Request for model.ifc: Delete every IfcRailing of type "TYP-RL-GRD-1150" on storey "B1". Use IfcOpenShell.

First a look at what the model holds.

```python
import ifcopenshell
import ifcopenshell.util.element

model = ifcopenshell.open("model.ifc")
print(model.schema)
storey = next(s for s in model.by_type("IfcBuildingStorey") if s.Name == "B1")
railings = [e for e in ifcopenshell.util.element.get_decomposition(storey) if e.is_a("IfcRailing")]
seen = {}
for e in railings:
    element_type = ifcopenshell.util.element.get_type(e)
    name = element_type.Name if element_type not in (None, e) else None
    seen[name] = seen.get(name, 0) + 1
for name, count in sorted(seen.items(), key=str):
    print(count, "x", name)
```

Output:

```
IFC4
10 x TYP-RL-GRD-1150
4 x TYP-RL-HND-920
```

```python
import ifcopenshell
import ifcopenshell.api.root
import ifcopenshell.util.element

model = ifcopenshell.open("model.ifc")

storey = next(s for s in model.by_type("IfcBuildingStorey") if s.Name == "B1")
railings = [e for e in ifcopenshell.util.element.get_decomposition(storey) if e.is_a("IfcRailing")]
targets = [e for e in railings if (t := ifcopenshell.util.element.get_type(e)) not in (None, e) and t.Name == "TYP-RL-GRD-1150"]

for e in targets:
    ifcopenshell.api.root.remove_product(model, product=e)
print(len(targets), "removed")

model.write("model_edited.ifc")
```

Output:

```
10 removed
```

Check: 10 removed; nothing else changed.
